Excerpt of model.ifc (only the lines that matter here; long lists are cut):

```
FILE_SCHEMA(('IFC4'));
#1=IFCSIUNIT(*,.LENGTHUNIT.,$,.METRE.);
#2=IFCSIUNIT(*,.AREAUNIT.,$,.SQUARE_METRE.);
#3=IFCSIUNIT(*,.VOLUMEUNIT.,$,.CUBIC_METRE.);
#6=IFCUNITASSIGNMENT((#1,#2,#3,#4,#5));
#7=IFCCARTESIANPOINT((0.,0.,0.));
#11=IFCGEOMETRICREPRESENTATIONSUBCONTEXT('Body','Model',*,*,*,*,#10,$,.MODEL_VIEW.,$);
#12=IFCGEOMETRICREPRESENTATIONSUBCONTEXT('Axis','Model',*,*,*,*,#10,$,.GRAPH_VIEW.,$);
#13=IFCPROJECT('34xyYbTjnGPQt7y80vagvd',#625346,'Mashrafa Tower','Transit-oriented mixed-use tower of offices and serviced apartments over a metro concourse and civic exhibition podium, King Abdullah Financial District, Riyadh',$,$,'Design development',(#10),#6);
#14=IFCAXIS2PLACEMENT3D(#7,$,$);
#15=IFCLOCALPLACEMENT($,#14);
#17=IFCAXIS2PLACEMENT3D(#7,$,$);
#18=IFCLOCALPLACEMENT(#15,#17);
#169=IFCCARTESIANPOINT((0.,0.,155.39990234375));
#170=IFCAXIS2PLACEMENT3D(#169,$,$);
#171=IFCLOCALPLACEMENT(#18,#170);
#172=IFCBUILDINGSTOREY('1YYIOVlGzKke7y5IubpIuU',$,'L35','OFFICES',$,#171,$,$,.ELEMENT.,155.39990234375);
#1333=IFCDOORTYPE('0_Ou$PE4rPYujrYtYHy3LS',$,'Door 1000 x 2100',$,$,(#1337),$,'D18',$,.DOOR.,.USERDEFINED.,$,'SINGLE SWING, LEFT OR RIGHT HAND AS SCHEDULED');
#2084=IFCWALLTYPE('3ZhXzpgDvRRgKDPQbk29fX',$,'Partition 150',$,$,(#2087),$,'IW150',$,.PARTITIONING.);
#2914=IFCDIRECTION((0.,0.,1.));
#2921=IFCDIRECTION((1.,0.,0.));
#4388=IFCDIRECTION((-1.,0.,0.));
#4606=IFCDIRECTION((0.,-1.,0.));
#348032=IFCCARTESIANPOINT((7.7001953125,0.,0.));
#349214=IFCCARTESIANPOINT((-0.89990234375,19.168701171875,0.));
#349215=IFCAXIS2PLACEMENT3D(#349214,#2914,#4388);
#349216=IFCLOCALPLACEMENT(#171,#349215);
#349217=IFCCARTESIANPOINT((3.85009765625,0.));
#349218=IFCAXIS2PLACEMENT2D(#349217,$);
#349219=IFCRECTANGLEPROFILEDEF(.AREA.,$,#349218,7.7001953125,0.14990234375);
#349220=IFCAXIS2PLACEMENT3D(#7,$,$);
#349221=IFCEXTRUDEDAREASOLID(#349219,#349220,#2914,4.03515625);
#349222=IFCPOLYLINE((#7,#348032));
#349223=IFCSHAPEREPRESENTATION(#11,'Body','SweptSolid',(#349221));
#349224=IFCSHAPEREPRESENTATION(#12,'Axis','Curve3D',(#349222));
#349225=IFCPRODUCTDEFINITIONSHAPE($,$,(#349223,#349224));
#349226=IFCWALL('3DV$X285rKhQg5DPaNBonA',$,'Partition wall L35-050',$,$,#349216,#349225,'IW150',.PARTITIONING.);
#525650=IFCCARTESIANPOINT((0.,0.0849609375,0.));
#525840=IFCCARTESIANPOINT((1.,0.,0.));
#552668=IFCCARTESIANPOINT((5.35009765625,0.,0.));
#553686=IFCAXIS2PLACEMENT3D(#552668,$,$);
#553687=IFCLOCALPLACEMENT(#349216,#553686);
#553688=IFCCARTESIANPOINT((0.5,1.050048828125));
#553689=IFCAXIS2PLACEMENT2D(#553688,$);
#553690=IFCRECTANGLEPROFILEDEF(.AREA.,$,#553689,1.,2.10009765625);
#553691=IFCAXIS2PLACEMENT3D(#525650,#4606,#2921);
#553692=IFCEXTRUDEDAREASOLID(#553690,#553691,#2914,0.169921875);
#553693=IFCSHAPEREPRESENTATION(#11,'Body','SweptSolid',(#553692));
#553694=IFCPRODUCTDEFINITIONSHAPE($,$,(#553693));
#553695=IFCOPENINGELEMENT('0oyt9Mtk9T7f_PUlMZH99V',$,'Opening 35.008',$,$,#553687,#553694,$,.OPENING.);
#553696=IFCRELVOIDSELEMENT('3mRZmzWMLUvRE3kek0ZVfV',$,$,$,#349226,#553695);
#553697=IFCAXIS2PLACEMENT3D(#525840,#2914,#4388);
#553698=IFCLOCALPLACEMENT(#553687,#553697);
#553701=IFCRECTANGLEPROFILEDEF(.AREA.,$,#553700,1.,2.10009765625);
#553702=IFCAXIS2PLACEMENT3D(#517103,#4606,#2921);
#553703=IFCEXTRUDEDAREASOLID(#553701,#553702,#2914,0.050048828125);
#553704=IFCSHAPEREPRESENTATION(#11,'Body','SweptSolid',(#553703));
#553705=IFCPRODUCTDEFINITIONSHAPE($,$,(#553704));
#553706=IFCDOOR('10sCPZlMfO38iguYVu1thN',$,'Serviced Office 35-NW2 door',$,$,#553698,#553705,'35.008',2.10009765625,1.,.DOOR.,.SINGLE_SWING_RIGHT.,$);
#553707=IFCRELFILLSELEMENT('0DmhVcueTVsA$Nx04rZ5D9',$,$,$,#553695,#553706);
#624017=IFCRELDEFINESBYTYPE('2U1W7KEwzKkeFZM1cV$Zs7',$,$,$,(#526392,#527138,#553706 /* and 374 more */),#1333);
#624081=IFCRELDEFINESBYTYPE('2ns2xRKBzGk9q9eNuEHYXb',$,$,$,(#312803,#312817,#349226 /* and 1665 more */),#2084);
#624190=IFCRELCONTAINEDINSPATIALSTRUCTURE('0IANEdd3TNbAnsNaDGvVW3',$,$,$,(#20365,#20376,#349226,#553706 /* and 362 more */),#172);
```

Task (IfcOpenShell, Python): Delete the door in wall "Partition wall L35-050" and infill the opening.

```python
import ifcopenshell
import ifcopenshell.api.feature
import ifcopenshell.api.root
import ifcopenshell.geom
import ifcopenshell.util.shape

model = ifcopenshell.open("model.ifc")
settings = ifcopenshell.geom.settings()


def volume(element):
    """Net volume in cubic metres, openings subtracted."""
    shape = ifcopenshell.geom.create_shape(settings, element)
    return ifcopenshell.util.shape.get_volume(shape.geometry)


door = model.by_guid("10sCPZlMfO38iguYVu1thN")
opening = door.FillsVoids[0].RelatingOpeningElement
wall = opening.VoidsElements[0].RelatingBuildingElement
before = volume(wall)

ifcopenshell.api.root.remove_product(model, product=door)
ifcopenshell.api.feature.remove_feature(model, feature=opening)

after = volume(wall)

print(f"wall volume {before:.3f} -> {after:.3f} m3")

model.write("model_updated.ifc")
```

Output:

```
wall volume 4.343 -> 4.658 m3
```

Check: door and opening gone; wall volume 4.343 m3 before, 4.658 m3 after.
